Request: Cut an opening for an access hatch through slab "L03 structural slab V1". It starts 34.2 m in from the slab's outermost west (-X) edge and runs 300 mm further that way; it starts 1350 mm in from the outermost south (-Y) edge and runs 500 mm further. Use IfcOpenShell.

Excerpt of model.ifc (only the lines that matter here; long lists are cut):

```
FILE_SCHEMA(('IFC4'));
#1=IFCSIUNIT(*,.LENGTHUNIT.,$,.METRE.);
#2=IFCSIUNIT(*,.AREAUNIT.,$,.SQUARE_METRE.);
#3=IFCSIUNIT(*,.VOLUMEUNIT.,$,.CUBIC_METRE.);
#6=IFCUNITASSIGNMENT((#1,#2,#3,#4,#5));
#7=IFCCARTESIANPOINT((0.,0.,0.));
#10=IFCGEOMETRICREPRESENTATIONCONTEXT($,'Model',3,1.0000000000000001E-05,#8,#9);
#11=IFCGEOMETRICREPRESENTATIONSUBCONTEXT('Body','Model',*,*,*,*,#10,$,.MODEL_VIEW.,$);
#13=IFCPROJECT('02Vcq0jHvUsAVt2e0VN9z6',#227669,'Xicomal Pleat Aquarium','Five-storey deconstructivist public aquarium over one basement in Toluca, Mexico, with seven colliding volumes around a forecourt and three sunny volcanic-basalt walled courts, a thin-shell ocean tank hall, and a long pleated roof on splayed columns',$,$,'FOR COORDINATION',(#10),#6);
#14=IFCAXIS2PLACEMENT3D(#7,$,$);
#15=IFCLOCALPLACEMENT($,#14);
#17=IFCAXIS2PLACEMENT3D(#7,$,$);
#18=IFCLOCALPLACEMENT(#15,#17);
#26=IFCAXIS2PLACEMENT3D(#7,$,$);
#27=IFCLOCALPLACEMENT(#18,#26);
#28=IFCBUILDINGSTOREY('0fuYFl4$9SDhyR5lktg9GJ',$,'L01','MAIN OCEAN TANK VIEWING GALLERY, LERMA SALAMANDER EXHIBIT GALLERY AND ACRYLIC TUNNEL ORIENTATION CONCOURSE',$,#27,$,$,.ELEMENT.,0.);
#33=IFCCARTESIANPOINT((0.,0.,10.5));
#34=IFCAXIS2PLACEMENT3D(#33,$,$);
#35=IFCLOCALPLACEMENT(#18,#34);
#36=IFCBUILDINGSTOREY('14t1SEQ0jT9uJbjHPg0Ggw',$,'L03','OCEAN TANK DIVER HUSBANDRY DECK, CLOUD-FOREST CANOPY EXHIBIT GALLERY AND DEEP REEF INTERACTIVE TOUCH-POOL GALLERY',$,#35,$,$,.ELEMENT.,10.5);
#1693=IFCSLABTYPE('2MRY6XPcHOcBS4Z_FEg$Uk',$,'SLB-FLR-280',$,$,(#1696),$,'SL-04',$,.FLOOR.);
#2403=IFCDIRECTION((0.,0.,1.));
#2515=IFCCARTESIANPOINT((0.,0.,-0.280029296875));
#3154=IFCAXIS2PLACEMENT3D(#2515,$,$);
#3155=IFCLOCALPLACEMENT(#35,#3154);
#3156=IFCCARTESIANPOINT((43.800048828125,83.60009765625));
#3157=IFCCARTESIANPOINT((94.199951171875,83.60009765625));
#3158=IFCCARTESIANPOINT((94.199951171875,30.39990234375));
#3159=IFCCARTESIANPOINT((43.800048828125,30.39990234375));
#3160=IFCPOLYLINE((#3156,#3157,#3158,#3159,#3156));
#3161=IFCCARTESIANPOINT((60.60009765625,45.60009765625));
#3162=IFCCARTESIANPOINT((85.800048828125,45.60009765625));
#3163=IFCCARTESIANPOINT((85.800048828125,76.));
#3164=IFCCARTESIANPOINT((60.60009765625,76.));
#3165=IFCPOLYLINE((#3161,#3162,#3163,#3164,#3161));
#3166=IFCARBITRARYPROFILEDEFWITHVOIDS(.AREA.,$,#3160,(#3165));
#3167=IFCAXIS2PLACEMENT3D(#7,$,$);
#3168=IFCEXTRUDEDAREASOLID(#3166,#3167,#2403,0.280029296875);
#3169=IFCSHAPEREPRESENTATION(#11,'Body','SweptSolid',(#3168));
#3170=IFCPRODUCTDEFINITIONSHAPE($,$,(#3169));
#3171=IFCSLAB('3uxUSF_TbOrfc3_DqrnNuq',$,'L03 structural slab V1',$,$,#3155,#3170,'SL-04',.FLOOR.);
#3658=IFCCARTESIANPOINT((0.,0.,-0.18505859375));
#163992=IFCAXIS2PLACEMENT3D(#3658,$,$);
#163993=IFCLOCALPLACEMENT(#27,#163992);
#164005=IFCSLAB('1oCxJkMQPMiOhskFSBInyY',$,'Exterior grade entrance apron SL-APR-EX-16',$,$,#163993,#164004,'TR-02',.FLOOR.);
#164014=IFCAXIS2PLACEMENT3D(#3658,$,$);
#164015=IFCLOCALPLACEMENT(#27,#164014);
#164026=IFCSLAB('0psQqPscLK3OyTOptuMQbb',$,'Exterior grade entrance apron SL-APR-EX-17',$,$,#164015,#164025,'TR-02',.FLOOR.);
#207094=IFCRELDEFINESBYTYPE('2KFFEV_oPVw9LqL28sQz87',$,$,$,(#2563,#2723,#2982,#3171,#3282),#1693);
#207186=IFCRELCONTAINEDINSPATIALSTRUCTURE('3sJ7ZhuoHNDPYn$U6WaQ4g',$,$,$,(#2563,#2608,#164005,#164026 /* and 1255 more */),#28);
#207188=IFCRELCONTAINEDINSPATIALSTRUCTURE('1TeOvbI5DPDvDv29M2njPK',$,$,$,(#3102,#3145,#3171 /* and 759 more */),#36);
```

```python
import numpy as np
import ifcopenshell
import ifcopenshell.api.feature
import ifcopenshell.api.geometry
import ifcopenshell.api.root
import ifcopenshell.geom
import ifcopenshell.util.placement
import ifcopenshell.util.representation
import ifcopenshell.util.shape
import ifcopenshell.util.unit

model = ifcopenshell.open("model.ifc")
unit_scale = ifcopenshell.util.unit.calculate_unit_scale(model)
settings = ifcopenshell.geom.settings()


def volume(element):
    """Net volume in cubic metres, openings subtracted."""
    shape = ifcopenshell.geom.create_shape(settings, element)
    return ifcopenshell.util.shape.get_volume(shape.geometry)


slab = model.by_guid("3uxUSF_TbOrfc3_DqrnNuq")
before = volume(slab)

# Extent in the slab's own axes, in metres. The edges named are its -X and -Y sides.
slab_shape = ifcopenshell.geom.create_shape(settings, slab)
vertices = ifcopenshell.util.shape.get_vertices(slab_shape.geometry)
x_min, y_min, bottom = vertices.min(axis=0)
top = vertices[:, 2].max()

opening = ifcopenshell.api.root.create_entity(model, ifc_class="IfcOpeningElement", name="Access hatch opening", predefined_type="OPENING")
context = ifcopenshell.util.representation.get_context(model, "Model", "Body", "MODEL_VIEW")
width, depth = 0.3, 0.5
outline = [(0.0, 0.0), (width, 0.0), (width, depth), (0.0, depth), (0.0, 0.0)]
# Overshoot both faces by 50 mm so the cut is clean.
shape = ifcopenshell.api.geometry.add_slab_representation(
    model, context=context, depth=top - bottom + 0.1, polyline=outline
)
ifcopenshell.api.geometry.assign_representation(model, product=opening, representation=shape)

matrix = ifcopenshell.util.placement.get_local_placement(slab.ObjectPlacement)
matrix[:, 3] = matrix @ np.append(np.array([x_min + 34.2, y_min + 1.35, bottom - 0.05]) / unit_scale, 1.0)
ifcopenshell.api.geometry.edit_object_placement(model, product=opening, matrix=matrix, is_si=False)
ifcopenshell.api.feature.add_feature(model, feature=opening, element=slab)

after = volume(slab)

print(f"slab volume {before:.3f} -> {after:.3f} m3")

model.write("model-out.ifc")
```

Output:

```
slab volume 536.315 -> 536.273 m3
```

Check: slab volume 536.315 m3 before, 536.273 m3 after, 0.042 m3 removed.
